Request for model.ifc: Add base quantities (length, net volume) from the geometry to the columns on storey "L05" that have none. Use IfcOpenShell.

First a look at what the model holds.

```python
import ifcopenshell
import ifcopenshell.util.element
import ifcopenshell.util.unit

model = ifcopenshell.open("model.ifc")
print(model.schema)
for unit_type in ("LENGTHUNIT", "AREAUNIT", "VOLUMEUNIT"):
    print(unit_type, ifcopenshell.util.unit.calculate_unit_scale(model, unit_type))
storey = next(s for s in model.by_type("IfcBuildingStorey") if s.Name == "L05")
columns = [e for e in ifcopenshell.util.element.get_decomposition(storey) if e.is_a("IfcColumn")]
for e in sorted(columns, key=lambda e: e.id()):
    print(e.id(), e.is_a(), e.Name, list(ifcopenshell.util.element.get_psets(e, qtos_only=True)), sep=" | ")
```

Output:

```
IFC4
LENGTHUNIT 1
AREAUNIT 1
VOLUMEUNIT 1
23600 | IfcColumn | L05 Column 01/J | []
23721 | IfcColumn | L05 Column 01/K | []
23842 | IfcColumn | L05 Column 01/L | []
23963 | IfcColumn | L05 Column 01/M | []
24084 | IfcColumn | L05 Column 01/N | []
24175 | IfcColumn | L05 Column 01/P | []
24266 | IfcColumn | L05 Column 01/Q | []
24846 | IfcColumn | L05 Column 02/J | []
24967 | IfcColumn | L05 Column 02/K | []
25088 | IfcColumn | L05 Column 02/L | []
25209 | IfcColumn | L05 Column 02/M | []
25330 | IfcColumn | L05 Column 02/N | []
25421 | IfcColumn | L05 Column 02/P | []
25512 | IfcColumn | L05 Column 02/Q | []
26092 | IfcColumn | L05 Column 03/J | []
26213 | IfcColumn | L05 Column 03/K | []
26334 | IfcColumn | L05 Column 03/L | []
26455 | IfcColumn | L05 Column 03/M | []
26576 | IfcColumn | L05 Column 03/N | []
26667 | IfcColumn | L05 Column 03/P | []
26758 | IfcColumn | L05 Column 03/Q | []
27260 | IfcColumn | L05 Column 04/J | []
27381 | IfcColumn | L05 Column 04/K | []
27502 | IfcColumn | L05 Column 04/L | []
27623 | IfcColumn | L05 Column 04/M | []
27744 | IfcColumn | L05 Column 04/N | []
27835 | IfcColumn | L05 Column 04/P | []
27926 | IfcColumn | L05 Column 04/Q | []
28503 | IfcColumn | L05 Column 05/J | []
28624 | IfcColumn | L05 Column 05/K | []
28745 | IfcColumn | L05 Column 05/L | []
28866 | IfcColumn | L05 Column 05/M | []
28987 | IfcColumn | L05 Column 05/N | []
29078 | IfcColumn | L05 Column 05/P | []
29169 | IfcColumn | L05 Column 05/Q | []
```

```python
import ifcopenshell
import ifcopenshell.api.pset
import ifcopenshell.geom
import ifcopenshell.util.element
import ifcopenshell.util.shape
import ifcopenshell.util.unit

model = ifcopenshell.open("model.ifc")
unit_scale = ifcopenshell.util.unit.calculate_unit_scale(model)
volume_scale = ifcopenshell.util.unit.calculate_unit_scale(model, "VOLUMEUNIT")
settings = ifcopenshell.geom.settings()

storey = next(s for s in model.by_type("IfcBuildingStorey") if s.Name == "L05")
columns = [e for e in ifcopenshell.util.element.get_decomposition(storey) if e.is_a("IfcColumn")]

for e in sorted(columns, key=lambda e: e.id()):
    if ifcopenshell.util.element.get_psets(e, qtos_only=True, should_inherit=False):
        continue
    # Geometry comes back in metres, in the element's own axes.
    shape = ifcopenshell.geom.create_shape(settings, e)
    values = {
        "Length": ifcopenshell.util.shape.get_z(shape.geometry) / unit_scale,
        "NetVolume": ifcopenshell.util.shape.get_volume(shape.geometry) / volume_scale,
    }
    qto = ifcopenshell.api.pset.add_qto(model, product=e, name="Qto_ColumnBaseQuantities")
    ifcopenshell.api.pset.edit_qto(model, qto=qto, properties=values)
    print(e.id(), {k: round(v, 3) for k, v in values.items()})

model.write("model_edited.ifc")
```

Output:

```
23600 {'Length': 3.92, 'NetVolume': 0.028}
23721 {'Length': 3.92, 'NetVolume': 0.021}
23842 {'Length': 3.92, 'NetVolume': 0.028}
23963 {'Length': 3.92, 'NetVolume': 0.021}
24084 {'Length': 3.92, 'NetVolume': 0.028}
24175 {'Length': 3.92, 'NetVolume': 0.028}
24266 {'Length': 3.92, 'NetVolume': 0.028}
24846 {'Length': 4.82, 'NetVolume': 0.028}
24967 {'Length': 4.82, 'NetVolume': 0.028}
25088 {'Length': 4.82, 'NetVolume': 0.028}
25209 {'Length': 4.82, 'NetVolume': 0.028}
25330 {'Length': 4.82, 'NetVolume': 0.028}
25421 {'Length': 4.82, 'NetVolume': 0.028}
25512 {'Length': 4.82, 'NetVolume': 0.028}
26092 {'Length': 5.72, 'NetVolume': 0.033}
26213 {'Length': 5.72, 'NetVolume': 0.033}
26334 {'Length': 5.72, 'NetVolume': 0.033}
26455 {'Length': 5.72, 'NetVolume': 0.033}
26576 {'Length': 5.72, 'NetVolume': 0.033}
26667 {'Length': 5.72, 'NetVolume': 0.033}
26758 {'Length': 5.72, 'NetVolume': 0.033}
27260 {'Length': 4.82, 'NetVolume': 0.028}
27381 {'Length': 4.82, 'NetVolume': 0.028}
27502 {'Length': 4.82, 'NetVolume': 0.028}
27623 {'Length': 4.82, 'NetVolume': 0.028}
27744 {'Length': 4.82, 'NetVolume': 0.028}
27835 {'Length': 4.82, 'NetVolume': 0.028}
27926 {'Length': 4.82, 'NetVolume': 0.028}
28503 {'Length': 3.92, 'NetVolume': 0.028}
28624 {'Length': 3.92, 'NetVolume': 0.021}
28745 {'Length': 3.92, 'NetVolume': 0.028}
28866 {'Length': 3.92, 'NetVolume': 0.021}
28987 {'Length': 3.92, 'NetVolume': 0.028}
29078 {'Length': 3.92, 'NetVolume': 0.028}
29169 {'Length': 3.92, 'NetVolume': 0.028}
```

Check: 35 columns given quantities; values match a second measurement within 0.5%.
